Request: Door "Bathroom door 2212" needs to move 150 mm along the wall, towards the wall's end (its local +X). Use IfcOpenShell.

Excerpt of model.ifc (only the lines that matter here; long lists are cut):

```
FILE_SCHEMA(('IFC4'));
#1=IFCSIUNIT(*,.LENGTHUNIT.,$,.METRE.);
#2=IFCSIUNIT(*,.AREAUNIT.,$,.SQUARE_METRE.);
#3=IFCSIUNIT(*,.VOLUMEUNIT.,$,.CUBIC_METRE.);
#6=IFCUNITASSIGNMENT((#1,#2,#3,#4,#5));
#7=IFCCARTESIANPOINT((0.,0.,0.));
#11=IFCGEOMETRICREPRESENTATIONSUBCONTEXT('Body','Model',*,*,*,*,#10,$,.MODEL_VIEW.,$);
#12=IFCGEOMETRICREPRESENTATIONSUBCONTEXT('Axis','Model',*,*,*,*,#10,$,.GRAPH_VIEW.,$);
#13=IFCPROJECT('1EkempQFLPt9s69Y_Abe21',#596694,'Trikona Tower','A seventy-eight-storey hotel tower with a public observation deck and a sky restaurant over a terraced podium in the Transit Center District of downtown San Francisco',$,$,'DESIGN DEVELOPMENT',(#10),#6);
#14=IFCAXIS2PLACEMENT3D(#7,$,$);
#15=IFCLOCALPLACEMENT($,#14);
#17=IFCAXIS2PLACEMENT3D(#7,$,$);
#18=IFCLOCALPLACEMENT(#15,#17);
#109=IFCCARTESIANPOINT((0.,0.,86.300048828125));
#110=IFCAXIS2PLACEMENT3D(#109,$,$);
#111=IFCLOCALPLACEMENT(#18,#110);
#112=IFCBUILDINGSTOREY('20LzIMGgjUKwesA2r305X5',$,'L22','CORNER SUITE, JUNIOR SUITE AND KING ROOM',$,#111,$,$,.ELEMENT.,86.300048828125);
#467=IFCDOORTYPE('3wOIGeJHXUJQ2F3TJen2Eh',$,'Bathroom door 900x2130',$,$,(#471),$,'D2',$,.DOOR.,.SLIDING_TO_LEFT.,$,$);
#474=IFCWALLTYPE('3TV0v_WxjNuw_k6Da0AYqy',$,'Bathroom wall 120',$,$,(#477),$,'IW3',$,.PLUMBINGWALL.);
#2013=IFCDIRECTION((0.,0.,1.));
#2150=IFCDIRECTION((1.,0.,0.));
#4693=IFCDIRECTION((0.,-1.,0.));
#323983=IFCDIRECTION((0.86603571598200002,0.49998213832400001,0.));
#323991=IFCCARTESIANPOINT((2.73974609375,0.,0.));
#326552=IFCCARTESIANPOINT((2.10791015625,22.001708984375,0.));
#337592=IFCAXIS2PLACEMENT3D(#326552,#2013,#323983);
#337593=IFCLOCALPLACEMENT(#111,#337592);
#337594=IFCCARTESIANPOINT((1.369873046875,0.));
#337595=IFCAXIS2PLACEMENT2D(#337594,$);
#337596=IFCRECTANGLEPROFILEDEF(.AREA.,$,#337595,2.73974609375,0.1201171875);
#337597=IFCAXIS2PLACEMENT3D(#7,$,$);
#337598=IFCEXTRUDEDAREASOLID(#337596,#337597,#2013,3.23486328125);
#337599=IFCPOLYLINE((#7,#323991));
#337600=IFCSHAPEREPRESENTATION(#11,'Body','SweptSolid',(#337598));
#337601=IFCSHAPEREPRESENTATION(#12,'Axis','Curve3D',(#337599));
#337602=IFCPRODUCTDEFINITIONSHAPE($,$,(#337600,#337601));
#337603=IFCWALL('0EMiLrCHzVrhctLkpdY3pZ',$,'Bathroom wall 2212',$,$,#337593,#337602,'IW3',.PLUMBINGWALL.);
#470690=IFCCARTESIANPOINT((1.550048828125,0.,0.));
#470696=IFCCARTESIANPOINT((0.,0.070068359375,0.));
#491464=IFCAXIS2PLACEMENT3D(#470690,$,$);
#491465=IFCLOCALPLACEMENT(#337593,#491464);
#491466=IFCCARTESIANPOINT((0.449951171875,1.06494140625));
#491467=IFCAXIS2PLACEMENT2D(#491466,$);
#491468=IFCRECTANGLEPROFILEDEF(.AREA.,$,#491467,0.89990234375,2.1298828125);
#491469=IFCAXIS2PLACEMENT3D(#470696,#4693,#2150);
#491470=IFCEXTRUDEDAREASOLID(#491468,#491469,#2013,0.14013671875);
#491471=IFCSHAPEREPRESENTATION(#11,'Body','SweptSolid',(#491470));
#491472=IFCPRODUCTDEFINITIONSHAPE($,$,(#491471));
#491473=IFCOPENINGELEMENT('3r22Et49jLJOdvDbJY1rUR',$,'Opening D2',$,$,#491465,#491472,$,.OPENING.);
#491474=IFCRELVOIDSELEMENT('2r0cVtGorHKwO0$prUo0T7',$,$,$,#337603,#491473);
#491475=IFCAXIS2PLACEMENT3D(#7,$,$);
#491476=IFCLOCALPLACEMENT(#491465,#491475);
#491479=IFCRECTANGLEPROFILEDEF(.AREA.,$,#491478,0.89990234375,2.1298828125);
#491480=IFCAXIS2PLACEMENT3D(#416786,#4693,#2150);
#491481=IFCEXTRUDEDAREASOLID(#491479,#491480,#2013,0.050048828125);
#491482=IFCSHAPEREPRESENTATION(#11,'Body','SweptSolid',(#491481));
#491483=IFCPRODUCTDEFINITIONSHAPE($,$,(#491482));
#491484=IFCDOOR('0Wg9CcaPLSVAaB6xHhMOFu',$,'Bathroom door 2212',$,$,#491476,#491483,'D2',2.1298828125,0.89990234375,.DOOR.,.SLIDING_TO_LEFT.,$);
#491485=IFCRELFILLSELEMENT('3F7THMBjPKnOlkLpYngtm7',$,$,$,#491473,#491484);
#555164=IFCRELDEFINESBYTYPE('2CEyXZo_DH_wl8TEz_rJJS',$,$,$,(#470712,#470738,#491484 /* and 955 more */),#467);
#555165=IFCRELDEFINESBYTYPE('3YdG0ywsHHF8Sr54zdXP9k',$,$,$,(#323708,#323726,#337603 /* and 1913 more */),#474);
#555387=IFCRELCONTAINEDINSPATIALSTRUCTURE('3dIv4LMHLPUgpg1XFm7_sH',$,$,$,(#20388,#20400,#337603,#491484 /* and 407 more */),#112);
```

```python
import ifcopenshell
import ifcopenshell.api.geometry
import ifcopenshell.util.placement

model = ifcopenshell.open("model.ifc")

door = model.by_guid("0Wg9CcaPLSVAaB6xHhMOFu")
opening = door.FillsVoids[0].RelatingOpeningElement
wall = opening.VoidsElements[0].RelatingBuildingElement

wall_matrix = ifcopenshell.util.placement.get_local_placement(wall.ObjectPlacement)
shift = wall_matrix[:3, 0] * 0.15
before = ifcopenshell.util.placement.get_local_placement(door.ObjectPlacement)[:3, 3].copy()

# The door is placed relative to its opening, so it follows when the opening moves.
matrix = ifcopenshell.util.placement.get_local_placement(opening.ObjectPlacement)
matrix[:3, 3] += shift
ifcopenshell.api.geometry.edit_object_placement(
    model, product=opening, matrix=matrix, is_si=False, should_transform_children=True
)

after = ifcopenshell.util.placement.get_local_placement(door.ObjectPlacement)[:3, 3]
print("door moved by", (after - before).round(3) + 0.0)

model.write("model_updated.ifc")
```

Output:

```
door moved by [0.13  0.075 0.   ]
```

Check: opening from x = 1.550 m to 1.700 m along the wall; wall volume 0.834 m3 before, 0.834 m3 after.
